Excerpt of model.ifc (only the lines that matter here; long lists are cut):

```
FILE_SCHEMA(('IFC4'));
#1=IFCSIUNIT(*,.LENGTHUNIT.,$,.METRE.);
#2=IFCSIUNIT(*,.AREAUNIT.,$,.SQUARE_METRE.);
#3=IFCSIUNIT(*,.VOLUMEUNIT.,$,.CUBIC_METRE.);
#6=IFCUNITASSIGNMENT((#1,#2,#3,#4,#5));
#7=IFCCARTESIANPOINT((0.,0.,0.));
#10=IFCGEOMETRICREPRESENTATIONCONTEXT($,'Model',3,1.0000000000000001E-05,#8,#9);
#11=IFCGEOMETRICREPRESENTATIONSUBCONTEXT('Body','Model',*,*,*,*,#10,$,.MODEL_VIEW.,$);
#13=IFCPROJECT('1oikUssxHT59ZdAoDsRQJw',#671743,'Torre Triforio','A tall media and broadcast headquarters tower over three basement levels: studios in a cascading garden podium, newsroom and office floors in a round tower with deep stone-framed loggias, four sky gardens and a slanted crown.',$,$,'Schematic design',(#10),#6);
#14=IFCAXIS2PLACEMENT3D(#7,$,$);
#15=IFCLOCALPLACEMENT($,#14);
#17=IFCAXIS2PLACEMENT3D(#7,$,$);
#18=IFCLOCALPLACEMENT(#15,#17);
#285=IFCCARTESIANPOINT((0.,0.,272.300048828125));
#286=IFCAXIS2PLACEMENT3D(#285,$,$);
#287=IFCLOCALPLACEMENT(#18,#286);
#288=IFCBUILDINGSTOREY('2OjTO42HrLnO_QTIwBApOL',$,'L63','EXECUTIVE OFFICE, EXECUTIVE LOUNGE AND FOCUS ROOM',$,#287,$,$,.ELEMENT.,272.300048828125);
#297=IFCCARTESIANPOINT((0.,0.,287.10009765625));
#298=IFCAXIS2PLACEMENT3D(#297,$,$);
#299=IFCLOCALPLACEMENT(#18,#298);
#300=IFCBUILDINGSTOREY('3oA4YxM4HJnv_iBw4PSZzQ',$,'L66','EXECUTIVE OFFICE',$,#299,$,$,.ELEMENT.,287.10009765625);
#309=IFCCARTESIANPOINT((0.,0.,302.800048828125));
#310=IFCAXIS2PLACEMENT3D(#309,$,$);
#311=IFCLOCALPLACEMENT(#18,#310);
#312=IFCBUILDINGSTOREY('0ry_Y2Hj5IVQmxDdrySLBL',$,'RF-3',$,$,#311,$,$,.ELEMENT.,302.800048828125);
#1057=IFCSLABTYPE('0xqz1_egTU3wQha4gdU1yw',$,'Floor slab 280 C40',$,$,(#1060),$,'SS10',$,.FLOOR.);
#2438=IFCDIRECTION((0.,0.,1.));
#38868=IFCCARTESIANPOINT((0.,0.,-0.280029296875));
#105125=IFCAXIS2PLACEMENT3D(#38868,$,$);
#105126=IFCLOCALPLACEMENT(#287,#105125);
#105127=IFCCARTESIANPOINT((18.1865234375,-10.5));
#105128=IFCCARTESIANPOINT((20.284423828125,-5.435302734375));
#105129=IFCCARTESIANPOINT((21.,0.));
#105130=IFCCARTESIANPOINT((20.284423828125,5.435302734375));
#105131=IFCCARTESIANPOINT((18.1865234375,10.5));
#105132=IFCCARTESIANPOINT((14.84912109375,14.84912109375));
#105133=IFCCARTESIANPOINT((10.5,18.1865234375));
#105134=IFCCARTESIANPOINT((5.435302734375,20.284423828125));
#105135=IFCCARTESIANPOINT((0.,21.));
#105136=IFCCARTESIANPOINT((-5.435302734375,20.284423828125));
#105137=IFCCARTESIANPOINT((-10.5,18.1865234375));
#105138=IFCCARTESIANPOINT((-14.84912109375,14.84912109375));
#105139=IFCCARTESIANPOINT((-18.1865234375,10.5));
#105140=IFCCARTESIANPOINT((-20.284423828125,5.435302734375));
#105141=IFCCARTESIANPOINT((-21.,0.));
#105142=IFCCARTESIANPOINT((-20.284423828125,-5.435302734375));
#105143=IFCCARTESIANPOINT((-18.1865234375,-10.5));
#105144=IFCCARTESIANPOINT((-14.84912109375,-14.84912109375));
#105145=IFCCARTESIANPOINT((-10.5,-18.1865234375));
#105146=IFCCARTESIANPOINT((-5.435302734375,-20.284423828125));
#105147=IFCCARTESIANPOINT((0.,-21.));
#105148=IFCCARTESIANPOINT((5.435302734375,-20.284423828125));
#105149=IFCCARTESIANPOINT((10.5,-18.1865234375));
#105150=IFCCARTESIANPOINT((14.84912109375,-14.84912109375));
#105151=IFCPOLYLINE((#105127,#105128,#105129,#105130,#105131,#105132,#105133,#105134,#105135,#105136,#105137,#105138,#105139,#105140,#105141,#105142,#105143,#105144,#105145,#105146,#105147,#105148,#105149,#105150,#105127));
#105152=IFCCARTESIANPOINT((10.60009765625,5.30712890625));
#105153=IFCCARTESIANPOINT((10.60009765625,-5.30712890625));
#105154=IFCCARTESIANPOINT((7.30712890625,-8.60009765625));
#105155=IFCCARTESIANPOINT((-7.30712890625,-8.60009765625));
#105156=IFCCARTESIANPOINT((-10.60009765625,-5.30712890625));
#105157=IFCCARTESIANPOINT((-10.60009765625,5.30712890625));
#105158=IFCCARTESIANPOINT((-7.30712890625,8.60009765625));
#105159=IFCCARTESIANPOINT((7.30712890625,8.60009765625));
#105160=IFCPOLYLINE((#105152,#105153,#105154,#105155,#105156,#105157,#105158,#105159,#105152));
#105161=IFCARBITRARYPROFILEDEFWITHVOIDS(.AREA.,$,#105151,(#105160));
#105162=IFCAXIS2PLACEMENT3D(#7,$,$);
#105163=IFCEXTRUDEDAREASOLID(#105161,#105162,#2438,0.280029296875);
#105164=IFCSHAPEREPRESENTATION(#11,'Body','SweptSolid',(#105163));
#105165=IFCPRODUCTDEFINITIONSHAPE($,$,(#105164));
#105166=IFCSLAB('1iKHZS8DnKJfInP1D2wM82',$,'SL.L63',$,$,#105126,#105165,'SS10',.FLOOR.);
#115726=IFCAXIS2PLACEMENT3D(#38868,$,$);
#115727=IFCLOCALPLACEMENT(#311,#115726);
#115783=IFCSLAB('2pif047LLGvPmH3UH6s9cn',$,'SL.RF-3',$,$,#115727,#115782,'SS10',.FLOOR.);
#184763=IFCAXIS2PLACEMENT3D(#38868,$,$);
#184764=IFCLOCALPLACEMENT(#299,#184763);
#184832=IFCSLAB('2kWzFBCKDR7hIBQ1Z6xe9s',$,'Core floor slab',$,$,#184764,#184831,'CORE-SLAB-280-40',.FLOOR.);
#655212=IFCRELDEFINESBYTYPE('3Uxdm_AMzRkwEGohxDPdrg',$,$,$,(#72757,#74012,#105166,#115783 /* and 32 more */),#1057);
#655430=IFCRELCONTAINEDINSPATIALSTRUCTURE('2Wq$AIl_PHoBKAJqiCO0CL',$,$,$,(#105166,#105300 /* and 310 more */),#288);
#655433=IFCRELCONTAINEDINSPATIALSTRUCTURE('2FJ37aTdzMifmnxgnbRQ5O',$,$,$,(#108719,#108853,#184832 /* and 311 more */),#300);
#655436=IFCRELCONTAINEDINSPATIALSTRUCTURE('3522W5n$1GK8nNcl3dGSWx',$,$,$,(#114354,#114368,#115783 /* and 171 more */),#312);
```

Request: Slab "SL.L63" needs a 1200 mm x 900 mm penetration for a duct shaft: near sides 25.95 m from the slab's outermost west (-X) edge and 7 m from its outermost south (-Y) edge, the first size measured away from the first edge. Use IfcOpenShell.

```python
import numpy as np
import ifcopenshell
import ifcopenshell.api.feature
import ifcopenshell.api.geometry
import ifcopenshell.api.root
import ifcopenshell.geom
import ifcopenshell.util.placement
import ifcopenshell.util.representation
import ifcopenshell.util.shape
import ifcopenshell.util.unit

model = ifcopenshell.open("model.ifc")
unit_scale = ifcopenshell.util.unit.calculate_unit_scale(model)
settings = ifcopenshell.geom.settings()


def volume(element):
    """Net volume in cubic metres, openings subtracted."""
    shape = ifcopenshell.geom.create_shape(settings, element)
    return ifcopenshell.util.shape.get_volume(shape.geometry)


slab = model.by_id(105166)
before = volume(slab)

# Extent in the slab's own axes, in metres. The edges named are its -X and -Y sides.
slab_shape = ifcopenshell.geom.create_shape(settings, slab)
vertices = ifcopenshell.util.shape.get_vertices(slab_shape.geometry)
x_min, y_min, bottom = vertices.min(axis=0)
top = vertices[:, 2].max()

opening = ifcopenshell.api.root.create_entity(model, ifc_class="IfcOpeningElement", name="Duct shaft opening", predefined_type="OPENING")
context = ifcopenshell.util.representation.get_context(model, "Model", "Body", "MODEL_VIEW")
width, depth = 1.2, 0.9
outline = [(0.0, 0.0), (width, 0.0), (width, depth), (0.0, depth), (0.0, 0.0)]
# Overshoot both faces by 50 mm so the cut is clean.
shape = ifcopenshell.api.geometry.add_slab_representation(
    model, context=context, depth=top - bottom + 0.1, polyline=outline
)
ifcopenshell.api.geometry.assign_representation(model, product=opening, representation=shape)

matrix = ifcopenshell.util.placement.get_local_placement(slab.ObjectPlacement)
matrix[:, 3] = matrix @ np.append(np.array([x_min + 25.95, y_min + 7, bottom - 0.05]) / unit_scale, 1.0)
ifcopenshell.api.geometry.edit_object_placement(model, product=opening, matrix=matrix, is_si=False)
ifcopenshell.api.feature.add_feature(model, feature=opening, element=slab)

after = volume(slab)

print(f"slab volume {before:.3f} -> {after:.3f} m3")

model.write("model_updated.ifc")
```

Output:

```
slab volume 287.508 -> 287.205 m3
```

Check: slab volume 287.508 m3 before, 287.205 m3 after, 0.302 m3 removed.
